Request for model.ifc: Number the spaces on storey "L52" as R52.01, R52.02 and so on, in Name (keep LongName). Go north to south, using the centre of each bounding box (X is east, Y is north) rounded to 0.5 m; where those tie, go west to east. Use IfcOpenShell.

First a look at what the model holds.

```python
import ifcopenshell
import ifcopenshell.util.element
import ifcopenshell.util.placement

model = ifcopenshell.open("model.ifc")
print(model.schema)
storey = next(s for s in model.by_type("IfcBuildingStorey") if s.Name == "L52")
spaces = [e for e in ifcopenshell.util.element.get_decomposition(storey) if e.is_a("IfcSpace")]
for e in sorted(spaces, key=lambda e: e.id()):
    origin = ifcopenshell.util.placement.get_local_placement(e.ObjectPlacement)[:3, 3]
    print(e.id(), e.Name, e.LongName, origin.round(2) + 0.0, sep=" | ")
```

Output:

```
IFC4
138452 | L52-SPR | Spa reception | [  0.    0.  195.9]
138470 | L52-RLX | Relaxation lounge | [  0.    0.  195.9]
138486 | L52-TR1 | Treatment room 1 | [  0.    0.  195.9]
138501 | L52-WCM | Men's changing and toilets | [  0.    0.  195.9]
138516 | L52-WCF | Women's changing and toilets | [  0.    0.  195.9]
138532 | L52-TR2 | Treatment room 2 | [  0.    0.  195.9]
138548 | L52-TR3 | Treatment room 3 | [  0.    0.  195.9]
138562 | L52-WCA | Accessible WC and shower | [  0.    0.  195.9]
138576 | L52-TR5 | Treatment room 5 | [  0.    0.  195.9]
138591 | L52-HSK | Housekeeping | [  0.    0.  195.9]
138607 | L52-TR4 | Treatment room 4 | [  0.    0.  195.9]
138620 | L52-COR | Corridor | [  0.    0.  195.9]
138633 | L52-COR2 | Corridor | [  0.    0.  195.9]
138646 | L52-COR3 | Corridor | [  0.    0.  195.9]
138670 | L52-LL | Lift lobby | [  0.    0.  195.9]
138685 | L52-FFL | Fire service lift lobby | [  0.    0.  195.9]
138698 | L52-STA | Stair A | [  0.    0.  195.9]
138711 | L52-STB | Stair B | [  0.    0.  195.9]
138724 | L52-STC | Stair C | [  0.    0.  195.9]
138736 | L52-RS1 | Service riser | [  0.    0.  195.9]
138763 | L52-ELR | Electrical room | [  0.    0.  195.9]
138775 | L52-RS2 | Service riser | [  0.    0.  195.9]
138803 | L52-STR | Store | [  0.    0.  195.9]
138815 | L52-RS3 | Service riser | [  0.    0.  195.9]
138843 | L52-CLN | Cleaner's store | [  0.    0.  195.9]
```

```python
import ifcopenshell
import ifcopenshell.geom
import ifcopenshell.util.element
import ifcopenshell.util.shape

model = ifcopenshell.open("model.ifc")
settings = ifcopenshell.geom.settings()
settings.set("use-world-coords", True)


def centre(element):
    shape = ifcopenshell.geom.create_shape(settings, element)
    return ifcopenshell.util.shape.get_bbox_centroid(shape.geometry)


storey = next(s for s in model.by_type("IfcBuildingStorey") if s.Name == "L52")
spaces = [e for e in ifcopenshell.util.element.get_decomposition(storey) if e.is_a("IfcSpace")]

# Insertion points can sit at a corner or the storey origin, so sort by the geometry (in metres).
centres = {e: centre(e) for e in spaces}
spaces.sort(key=lambda e: (-round(centres[e][1] / 0.5), centres[e][0]))

for i, e in enumerate(spaces, start=1):
    number = f"R52.{i:02d}"
    e.Name = number
    print(e.id(), number)

model.write("model_v2.ifc")
```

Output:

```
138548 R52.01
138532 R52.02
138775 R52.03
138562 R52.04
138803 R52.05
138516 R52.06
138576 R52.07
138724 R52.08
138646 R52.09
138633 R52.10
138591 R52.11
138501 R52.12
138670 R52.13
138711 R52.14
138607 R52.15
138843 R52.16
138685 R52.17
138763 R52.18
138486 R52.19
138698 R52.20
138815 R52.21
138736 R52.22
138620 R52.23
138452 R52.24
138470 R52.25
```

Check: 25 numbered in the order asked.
